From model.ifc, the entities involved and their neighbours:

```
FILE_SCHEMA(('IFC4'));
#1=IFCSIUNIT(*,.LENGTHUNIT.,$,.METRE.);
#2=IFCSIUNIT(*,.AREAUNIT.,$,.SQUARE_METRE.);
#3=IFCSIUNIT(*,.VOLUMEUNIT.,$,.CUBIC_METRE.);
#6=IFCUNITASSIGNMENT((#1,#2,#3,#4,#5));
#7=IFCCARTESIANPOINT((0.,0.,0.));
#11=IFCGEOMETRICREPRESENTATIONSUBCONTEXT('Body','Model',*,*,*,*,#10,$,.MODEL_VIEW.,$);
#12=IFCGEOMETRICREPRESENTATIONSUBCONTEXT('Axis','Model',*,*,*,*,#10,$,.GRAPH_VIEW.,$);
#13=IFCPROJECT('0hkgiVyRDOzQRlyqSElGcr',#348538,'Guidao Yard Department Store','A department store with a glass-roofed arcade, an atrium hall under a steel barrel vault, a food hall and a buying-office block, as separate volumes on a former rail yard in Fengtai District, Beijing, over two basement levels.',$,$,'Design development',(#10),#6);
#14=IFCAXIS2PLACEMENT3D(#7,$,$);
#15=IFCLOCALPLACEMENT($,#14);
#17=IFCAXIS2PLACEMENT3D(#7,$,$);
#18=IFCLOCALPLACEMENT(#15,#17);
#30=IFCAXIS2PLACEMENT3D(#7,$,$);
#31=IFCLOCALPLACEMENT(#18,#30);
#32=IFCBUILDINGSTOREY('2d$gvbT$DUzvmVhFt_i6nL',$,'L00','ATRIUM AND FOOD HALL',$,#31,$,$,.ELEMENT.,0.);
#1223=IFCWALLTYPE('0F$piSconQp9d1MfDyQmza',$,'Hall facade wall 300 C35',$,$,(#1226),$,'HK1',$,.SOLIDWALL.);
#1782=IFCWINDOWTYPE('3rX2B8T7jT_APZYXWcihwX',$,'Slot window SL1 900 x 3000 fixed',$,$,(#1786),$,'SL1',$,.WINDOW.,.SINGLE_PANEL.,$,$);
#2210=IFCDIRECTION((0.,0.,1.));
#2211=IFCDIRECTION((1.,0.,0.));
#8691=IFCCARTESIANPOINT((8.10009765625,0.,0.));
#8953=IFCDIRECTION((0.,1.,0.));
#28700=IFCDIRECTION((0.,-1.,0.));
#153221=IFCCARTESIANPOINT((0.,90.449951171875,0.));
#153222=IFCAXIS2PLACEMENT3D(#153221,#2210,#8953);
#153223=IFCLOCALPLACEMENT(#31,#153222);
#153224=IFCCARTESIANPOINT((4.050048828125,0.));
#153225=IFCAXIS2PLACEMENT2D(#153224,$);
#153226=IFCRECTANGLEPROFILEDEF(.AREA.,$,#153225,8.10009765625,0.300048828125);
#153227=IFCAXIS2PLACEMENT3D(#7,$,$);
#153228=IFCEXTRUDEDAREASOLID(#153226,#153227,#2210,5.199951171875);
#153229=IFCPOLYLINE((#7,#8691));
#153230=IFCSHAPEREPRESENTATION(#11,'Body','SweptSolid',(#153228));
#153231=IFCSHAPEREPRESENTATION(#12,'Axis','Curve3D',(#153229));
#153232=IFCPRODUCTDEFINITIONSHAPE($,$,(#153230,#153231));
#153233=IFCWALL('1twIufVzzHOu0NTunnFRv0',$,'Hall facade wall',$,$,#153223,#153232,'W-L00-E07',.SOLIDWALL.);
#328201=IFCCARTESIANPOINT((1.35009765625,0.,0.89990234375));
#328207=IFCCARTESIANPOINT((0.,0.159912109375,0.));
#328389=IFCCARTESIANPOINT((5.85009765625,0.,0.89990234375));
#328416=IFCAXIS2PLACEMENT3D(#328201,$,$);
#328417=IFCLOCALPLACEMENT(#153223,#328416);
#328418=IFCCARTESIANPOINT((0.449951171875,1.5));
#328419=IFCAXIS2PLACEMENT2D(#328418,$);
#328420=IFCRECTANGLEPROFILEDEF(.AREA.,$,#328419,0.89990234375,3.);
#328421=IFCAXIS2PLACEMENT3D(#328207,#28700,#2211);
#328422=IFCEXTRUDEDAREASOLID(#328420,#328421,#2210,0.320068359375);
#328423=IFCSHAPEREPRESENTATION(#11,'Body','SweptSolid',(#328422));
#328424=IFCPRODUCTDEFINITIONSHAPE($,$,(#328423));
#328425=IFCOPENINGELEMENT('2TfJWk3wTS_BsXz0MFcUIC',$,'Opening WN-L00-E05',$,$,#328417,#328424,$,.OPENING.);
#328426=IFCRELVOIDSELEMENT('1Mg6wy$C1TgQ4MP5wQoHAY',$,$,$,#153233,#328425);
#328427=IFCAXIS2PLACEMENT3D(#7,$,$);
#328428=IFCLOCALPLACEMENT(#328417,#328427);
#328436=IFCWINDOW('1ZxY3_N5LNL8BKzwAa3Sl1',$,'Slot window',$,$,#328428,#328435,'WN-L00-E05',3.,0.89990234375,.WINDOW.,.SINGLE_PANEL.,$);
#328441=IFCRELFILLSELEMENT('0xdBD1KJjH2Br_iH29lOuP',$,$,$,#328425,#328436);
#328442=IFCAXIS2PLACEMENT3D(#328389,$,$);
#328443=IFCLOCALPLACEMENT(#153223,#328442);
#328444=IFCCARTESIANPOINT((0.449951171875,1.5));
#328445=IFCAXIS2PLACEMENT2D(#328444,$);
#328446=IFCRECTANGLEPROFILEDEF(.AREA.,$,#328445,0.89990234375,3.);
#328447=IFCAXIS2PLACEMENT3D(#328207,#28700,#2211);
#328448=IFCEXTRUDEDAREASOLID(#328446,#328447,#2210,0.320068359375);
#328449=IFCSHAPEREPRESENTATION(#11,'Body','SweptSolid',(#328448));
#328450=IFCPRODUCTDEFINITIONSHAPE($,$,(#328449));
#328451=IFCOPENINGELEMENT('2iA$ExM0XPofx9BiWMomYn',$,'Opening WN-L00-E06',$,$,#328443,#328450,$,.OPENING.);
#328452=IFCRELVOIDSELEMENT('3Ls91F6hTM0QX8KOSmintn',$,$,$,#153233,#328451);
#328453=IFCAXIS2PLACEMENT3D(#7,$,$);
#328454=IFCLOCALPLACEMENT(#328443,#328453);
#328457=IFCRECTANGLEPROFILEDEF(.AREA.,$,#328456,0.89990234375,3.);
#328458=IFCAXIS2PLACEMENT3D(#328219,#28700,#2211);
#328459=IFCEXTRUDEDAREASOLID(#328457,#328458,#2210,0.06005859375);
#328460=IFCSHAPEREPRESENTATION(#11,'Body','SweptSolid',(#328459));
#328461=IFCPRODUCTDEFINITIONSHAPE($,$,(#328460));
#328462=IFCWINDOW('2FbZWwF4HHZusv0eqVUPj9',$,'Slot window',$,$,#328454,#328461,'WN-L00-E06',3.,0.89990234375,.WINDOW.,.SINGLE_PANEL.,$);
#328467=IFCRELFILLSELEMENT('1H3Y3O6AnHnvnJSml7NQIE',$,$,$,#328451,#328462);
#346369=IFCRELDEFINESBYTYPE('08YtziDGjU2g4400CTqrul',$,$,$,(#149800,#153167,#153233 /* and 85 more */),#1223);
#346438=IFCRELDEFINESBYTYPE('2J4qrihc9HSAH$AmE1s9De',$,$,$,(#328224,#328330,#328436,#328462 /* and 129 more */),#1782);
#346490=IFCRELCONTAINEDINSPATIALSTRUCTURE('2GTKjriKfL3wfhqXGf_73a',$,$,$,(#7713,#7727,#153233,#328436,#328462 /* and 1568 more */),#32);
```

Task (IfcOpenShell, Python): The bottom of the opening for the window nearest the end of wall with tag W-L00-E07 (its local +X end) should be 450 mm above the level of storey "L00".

```python
import numpy as np
import ifcopenshell
import ifcopenshell.api.geometry
import ifcopenshell.geom
import ifcopenshell.util.element
import ifcopenshell.util.placement
import ifcopenshell.util.shape
import ifcopenshell.util.unit

model = ifcopenshell.open("model.ifc")
unit_scale = ifcopenshell.util.unit.calculate_unit_scale(model)

window = model.by_id(328462)
opening = window.FillsVoids[0].RelatingOpeningElement
storey = ifcopenshell.util.element.get_container(window, ifc_class="IfcBuildingStorey")
level = ifcopenshell.util.placement.get_local_placement(storey.ObjectPlacement)[2, 3]

# The opening's origin need not be at the sill, so measure its lowest point.
shape = ifcopenshell.geom.create_shape(ifcopenshell.geom.settings(), opening)
bottom = ifcopenshell.util.shape.get_shape_bottom_elevation(shape, shape.geometry) / unit_scale
dz = level + 0.45 / unit_scale - bottom

shift = np.array([0.0, 0.0, dz])
# The window is placed relative to its opening, so it follows when the opening moves.
matrix = ifcopenshell.util.placement.get_local_placement(opening.ObjectPlacement)
matrix[:3, 3] += shift
ifcopenshell.api.geometry.edit_object_placement(
    model, product=opening, matrix=matrix, is_si=False, should_transform_children=True
)

print(f"moved by {dz * unit_scale:+.3f} m")

model.write("model_rev.ifc")
```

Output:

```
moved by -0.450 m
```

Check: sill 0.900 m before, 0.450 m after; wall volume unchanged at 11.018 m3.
